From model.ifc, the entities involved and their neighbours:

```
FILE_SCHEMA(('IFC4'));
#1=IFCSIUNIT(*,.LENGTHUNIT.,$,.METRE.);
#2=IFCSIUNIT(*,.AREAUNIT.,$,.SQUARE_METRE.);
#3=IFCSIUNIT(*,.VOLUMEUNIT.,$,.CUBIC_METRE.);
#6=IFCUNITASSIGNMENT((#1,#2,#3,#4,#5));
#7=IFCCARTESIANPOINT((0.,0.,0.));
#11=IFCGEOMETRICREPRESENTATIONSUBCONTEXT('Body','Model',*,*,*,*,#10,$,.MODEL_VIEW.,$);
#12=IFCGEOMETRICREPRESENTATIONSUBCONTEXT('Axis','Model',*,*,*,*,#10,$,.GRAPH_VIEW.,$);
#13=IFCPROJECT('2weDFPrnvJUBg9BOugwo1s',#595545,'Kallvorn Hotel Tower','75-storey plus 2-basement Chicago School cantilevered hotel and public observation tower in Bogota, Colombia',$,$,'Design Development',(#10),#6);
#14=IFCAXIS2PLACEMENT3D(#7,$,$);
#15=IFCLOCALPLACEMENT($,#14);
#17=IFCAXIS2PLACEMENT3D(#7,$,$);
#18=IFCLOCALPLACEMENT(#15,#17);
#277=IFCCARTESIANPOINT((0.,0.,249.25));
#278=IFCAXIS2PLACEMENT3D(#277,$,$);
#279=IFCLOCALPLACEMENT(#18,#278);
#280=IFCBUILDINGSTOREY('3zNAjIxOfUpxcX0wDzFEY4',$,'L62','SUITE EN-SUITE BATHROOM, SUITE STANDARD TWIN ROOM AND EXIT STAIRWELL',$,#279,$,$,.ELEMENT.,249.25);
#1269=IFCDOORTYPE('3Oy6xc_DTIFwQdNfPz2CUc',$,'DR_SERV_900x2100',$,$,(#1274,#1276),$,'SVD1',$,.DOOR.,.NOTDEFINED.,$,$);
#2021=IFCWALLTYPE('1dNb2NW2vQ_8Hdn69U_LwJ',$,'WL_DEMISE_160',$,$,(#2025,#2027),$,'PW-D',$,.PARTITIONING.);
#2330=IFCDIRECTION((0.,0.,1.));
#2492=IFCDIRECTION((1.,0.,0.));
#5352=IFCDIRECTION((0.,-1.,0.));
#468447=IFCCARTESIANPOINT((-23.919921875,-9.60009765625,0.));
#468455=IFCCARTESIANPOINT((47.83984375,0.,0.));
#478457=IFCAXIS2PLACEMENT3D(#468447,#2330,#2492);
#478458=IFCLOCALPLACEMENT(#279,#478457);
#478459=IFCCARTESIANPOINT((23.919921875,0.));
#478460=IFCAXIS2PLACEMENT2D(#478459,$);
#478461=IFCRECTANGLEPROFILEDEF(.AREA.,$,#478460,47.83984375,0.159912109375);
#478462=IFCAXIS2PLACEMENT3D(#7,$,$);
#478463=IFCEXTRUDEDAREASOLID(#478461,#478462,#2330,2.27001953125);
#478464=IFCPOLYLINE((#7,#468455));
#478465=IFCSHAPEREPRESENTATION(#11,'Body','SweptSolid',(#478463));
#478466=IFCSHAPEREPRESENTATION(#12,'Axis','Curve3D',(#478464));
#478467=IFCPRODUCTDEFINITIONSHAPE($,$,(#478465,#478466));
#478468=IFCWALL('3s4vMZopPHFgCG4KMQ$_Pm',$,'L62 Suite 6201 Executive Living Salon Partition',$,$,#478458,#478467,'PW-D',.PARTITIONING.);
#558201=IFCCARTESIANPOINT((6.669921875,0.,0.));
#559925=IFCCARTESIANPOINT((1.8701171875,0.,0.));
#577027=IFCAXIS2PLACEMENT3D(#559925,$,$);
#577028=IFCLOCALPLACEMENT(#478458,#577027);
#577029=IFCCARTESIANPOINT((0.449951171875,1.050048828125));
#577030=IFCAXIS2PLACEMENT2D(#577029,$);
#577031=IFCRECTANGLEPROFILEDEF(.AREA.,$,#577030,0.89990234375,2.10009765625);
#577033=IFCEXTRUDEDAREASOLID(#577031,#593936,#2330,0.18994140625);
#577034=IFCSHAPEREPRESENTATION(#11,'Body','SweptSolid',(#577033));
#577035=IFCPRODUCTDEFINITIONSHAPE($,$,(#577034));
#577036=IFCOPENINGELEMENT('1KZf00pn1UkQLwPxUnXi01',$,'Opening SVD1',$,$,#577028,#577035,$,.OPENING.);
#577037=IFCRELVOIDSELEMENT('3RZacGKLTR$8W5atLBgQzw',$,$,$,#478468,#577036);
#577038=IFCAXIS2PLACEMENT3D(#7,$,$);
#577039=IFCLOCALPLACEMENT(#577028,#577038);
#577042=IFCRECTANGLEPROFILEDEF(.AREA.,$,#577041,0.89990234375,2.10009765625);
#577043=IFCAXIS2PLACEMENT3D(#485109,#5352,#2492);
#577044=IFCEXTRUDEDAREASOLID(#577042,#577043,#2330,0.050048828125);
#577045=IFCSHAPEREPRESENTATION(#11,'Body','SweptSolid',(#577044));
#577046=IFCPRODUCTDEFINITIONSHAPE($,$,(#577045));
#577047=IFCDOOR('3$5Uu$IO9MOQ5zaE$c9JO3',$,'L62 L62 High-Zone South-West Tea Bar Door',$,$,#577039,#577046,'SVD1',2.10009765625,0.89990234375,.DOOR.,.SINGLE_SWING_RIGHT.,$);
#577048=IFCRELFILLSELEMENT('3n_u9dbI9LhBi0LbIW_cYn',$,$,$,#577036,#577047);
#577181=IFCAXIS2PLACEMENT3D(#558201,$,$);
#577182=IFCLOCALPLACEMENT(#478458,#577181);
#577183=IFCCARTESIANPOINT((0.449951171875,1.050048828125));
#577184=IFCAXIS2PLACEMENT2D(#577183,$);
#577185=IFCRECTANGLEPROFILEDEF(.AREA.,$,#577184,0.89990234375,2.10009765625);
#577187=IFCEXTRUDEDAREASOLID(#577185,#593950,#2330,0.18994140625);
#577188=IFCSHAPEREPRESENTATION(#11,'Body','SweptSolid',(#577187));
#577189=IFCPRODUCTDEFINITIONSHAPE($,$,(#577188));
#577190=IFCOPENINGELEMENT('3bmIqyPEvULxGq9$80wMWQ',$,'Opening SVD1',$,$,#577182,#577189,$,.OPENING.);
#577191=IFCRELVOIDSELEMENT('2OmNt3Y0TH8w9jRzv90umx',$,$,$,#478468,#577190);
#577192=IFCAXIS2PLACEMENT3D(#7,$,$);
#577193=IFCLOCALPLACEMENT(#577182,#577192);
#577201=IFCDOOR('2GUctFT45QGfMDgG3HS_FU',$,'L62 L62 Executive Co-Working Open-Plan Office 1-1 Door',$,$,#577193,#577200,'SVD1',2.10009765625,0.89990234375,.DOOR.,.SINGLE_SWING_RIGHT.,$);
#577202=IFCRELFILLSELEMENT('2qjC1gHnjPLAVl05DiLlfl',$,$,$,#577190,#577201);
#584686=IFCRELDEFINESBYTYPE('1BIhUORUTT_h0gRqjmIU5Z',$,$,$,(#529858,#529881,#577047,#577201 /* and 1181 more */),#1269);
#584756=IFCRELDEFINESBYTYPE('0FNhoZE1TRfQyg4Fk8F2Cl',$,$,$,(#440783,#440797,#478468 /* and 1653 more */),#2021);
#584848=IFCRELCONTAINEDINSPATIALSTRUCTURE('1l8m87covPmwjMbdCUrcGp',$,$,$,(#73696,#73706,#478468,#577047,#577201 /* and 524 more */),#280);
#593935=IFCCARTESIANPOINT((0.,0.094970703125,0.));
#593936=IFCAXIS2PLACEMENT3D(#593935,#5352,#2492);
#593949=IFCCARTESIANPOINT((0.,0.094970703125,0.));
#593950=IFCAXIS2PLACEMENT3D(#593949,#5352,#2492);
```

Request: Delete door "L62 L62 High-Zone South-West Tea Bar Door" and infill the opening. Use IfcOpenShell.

```python
import ifcopenshell
import ifcopenshell.api.feature
import ifcopenshell.api.root
import ifcopenshell.geom
import ifcopenshell.util.shape

model = ifcopenshell.open("model.ifc")
settings = ifcopenshell.geom.settings()


def volume(element):
    """Net volume in cubic metres, openings subtracted."""
    shape = ifcopenshell.geom.create_shape(settings, element)
    return ifcopenshell.util.shape.get_volume(shape.geometry)


door = model.by_guid("3$5Uu$IO9MOQ5zaE$c9JO3")
opening = door.FillsVoids[0].RelatingOpeningElement
wall = opening.VoidsElements[0].RelatingBuildingElement
before = volume(wall)

ifcopenshell.api.root.remove_product(model, product=door)
ifcopenshell.api.feature.remove_feature(model, feature=opening)

after = volume(wall)

print(f"wall volume {before:.3f} -> {after:.3f} m3")

model.write("model_edited.ifc")
```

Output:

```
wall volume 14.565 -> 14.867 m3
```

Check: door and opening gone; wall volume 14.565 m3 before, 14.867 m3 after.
